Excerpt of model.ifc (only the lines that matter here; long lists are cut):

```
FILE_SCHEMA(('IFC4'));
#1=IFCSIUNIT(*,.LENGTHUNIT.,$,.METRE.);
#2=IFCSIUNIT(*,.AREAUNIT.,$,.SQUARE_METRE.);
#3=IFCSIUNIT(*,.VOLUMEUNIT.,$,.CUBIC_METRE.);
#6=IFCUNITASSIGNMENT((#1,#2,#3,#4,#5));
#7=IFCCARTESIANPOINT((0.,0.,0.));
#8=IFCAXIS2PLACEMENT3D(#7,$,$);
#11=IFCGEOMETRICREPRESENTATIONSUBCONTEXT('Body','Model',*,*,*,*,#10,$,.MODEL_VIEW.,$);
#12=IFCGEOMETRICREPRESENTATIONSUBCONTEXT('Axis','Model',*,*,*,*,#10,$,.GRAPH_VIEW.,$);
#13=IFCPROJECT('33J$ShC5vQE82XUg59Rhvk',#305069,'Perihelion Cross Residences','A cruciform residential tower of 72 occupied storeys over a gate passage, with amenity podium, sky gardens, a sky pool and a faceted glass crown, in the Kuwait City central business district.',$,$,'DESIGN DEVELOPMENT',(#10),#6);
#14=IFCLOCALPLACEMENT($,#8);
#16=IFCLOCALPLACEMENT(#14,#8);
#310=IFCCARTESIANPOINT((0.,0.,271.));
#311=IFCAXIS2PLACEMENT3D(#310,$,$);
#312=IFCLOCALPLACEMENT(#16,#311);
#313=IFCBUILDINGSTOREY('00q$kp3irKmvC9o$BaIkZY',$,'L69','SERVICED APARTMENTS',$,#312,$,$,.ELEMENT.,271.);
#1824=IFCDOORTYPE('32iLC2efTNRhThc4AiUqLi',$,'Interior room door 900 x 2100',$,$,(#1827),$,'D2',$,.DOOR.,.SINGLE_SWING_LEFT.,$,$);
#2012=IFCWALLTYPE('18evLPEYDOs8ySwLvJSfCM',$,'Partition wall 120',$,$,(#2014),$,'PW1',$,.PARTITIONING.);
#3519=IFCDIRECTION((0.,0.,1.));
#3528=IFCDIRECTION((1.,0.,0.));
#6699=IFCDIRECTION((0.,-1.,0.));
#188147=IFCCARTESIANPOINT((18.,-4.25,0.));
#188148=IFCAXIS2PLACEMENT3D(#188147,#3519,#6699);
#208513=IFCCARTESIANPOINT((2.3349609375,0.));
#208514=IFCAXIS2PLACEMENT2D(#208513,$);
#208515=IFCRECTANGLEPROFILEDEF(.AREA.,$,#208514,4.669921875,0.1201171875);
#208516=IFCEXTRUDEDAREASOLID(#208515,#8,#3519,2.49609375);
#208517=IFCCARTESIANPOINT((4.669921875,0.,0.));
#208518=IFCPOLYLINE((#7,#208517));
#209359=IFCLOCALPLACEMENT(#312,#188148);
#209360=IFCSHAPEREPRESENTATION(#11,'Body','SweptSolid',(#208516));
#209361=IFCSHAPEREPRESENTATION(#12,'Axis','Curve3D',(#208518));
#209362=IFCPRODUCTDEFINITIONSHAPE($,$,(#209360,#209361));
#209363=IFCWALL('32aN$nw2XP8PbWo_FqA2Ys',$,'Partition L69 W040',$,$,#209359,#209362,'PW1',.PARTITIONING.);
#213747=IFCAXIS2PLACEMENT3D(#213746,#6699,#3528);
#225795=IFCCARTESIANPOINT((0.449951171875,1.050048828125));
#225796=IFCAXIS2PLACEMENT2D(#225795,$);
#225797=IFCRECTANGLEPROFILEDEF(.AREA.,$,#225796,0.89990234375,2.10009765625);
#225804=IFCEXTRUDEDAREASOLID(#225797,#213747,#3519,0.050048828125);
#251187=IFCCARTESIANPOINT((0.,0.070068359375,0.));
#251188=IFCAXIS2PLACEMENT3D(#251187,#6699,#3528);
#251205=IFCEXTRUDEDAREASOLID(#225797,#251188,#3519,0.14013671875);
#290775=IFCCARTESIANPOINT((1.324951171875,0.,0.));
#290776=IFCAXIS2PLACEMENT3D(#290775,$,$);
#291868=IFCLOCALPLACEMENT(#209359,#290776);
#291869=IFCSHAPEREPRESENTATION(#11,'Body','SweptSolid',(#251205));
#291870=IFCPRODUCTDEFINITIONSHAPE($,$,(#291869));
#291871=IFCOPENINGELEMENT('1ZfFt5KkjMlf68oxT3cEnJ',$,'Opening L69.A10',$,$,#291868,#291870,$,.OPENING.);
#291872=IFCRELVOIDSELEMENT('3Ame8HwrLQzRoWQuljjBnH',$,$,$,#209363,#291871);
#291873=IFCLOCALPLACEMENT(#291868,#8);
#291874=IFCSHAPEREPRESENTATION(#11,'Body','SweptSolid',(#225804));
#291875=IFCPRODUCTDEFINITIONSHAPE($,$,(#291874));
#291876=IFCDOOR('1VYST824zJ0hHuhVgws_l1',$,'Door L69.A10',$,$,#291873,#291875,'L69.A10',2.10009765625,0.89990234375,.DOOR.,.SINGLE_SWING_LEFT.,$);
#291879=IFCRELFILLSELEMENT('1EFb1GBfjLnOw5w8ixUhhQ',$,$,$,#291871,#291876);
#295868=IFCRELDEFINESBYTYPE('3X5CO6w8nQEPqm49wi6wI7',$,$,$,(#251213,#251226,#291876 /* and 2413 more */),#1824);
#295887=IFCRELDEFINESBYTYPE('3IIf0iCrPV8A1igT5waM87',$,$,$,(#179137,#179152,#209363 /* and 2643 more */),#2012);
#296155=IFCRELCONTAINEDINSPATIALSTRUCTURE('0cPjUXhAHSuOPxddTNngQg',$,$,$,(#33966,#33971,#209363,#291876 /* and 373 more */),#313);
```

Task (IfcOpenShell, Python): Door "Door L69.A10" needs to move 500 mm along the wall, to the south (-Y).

```python
import ifcopenshell
import ifcopenshell.api.geometry
import ifcopenshell.util.placement
import ifcopenshell.util.unit

model = ifcopenshell.open("model.ifc")
unit_scale = ifcopenshell.util.unit.calculate_unit_scale(model)

door = model.by_guid("1VYST824zJ0hHuhVgws_l1")
opening = door.FillsVoids[0].RelatingOpeningElement
wall = opening.VoidsElements[0].RelatingBuildingElement

wall_matrix = ifcopenshell.util.placement.get_local_placement(wall.ObjectPlacement)
shift = wall_matrix[:3, 0] * 0.5 / unit_scale
before = ifcopenshell.util.placement.get_local_placement(door.ObjectPlacement)[:3, 3].copy()

# The door is placed relative to its opening, so it follows when the opening moves.
matrix = ifcopenshell.util.placement.get_local_placement(opening.ObjectPlacement)
matrix[:3, 3] += shift
ifcopenshell.api.geometry.edit_object_placement(
    model, product=opening, matrix=matrix, is_si=False, should_transform_children=True
)

after = ifcopenshell.util.placement.get_local_placement(door.ObjectPlacement)[:3, 3]
print("door moved by", (after - before).round(3) + 0.0)

model.write("model_v2.ifc")
```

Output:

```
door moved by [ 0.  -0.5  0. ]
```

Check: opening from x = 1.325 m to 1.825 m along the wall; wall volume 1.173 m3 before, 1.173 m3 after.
